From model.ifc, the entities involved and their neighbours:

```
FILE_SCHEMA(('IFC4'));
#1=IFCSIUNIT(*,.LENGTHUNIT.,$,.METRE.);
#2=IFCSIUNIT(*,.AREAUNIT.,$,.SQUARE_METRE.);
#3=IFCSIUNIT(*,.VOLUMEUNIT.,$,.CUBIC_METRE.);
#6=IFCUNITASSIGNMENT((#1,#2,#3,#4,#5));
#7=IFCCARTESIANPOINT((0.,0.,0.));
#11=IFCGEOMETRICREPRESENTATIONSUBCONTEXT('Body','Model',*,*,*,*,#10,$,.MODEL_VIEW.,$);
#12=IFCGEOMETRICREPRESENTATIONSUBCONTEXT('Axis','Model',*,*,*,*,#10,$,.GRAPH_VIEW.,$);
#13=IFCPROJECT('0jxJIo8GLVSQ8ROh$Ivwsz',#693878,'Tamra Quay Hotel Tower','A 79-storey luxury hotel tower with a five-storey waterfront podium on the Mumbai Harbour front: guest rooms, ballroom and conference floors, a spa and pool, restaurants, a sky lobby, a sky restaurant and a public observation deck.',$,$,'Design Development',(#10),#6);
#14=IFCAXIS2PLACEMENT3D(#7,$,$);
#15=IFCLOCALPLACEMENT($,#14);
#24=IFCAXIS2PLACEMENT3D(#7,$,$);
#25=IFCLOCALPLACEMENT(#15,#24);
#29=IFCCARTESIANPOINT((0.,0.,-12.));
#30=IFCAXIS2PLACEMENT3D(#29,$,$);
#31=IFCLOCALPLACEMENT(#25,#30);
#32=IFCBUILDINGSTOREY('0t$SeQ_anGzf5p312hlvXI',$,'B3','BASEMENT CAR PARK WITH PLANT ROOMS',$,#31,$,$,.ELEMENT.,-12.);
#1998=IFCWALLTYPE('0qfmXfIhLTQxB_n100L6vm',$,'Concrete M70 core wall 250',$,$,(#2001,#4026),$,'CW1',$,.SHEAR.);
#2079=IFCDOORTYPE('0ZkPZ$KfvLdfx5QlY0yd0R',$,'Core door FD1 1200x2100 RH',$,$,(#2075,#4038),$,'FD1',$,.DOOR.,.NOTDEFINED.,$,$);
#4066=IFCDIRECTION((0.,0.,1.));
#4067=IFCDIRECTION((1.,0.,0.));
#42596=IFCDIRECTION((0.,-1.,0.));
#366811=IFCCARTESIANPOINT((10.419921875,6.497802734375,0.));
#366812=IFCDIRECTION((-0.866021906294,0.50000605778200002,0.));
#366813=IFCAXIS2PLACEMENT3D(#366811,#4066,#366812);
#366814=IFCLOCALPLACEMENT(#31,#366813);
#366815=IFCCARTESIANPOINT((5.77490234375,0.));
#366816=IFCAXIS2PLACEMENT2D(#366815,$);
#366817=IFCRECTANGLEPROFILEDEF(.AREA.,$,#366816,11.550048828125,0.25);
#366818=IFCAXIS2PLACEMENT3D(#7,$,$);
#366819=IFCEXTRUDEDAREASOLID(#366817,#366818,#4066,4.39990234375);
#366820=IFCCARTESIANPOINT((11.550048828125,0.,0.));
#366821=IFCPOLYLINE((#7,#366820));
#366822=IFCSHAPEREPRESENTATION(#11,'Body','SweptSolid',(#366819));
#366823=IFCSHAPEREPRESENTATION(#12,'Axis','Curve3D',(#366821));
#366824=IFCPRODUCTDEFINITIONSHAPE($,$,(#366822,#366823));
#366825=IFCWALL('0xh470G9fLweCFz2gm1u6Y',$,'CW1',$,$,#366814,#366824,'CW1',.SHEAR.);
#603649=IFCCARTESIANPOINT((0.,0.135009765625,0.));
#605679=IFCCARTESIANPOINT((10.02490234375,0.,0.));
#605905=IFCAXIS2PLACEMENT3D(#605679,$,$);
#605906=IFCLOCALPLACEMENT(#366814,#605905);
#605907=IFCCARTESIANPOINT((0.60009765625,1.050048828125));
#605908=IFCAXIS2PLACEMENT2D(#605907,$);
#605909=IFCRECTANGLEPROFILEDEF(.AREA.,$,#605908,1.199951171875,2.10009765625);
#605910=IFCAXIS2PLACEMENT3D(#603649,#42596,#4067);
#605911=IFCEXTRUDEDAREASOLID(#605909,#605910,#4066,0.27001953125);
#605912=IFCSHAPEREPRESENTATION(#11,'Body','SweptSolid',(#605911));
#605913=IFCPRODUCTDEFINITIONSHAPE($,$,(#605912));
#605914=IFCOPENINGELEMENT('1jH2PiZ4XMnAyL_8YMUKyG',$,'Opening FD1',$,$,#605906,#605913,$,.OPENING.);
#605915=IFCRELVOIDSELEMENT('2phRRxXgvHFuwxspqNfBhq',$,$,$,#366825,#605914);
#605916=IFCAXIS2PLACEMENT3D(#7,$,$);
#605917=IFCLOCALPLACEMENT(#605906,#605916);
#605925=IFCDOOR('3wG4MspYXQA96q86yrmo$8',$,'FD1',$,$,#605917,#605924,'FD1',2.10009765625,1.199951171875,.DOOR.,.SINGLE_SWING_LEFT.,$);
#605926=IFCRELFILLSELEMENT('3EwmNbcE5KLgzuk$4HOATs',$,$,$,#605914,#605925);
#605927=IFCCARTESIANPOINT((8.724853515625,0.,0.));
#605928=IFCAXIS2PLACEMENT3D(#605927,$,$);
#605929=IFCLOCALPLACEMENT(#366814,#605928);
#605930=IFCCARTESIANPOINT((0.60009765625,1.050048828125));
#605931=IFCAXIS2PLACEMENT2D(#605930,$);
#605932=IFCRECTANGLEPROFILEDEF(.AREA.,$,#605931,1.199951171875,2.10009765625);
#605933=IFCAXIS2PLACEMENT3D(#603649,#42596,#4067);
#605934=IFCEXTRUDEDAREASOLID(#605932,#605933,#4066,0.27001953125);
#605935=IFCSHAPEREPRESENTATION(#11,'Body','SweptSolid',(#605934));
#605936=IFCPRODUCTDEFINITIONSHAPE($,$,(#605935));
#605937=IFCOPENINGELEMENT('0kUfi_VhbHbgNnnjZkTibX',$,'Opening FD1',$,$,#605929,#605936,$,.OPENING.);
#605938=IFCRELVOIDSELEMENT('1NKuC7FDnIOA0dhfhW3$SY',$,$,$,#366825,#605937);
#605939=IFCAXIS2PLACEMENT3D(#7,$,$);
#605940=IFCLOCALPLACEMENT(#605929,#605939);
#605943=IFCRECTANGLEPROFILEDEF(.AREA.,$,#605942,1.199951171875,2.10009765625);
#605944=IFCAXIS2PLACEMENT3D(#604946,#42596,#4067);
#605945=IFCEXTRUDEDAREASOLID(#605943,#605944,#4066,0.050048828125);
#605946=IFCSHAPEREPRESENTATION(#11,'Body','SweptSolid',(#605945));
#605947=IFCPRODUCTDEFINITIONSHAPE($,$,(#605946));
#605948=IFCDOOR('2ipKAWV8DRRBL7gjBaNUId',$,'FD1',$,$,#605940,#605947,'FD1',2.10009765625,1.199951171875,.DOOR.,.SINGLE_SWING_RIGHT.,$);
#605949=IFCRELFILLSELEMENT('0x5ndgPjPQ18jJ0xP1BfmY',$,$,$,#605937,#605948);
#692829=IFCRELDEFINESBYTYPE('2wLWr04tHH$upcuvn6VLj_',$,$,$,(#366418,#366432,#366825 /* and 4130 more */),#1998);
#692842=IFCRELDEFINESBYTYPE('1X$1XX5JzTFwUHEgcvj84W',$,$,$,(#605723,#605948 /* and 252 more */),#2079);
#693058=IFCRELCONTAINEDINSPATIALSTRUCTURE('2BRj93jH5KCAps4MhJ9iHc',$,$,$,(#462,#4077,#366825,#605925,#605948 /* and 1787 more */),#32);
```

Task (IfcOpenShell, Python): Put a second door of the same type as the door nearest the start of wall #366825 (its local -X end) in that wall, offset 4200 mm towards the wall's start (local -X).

```python
import ifcopenshell
import ifcopenshell.api.feature
import ifcopenshell.api.geometry
import ifcopenshell.api.root
import ifcopenshell.geom
import ifcopenshell.util.element
import ifcopenshell.util.placement
import ifcopenshell.util.shape
import ifcopenshell.util.unit

model = ifcopenshell.open("model.ifc")
unit_scale = ifcopenshell.util.unit.calculate_unit_scale(model)
settings = ifcopenshell.geom.settings()


def volume(element):
    """Net volume in cubic metres, openings subtracted."""
    shape = ifcopenshell.geom.create_shape(settings, element)
    return ifcopenshell.util.shape.get_volume(shape.geometry)


door = model.by_guid("2ipKAWV8DRRBL7gjBaNUId")
opening = door.FillsVoids[0].RelatingOpeningElement
wall = opening.VoidsElements[0].RelatingBuildingElement
before = volume(wall)
shift = ifcopenshell.util.placement.get_local_placement(wall.ObjectPlacement)[:3, 0] * -4.2 / unit_scale

# copy_class copies the void relationship, type, container and properties, but no geometry.
new_opening = ifcopenshell.api.root.copy_class(model, product=opening)
new_opening.Representation = ifcopenshell.util.element.copy_deep(
    model, opening.Representation, exclude=["IfcGeometricRepresentationContext", "IfcRepresentationMap"]
)
new_door = ifcopenshell.api.root.copy_class(model, product=door)
new_door.Representation = ifcopenshell.util.element.copy_deep(
    model, door.Representation, exclude=["IfcGeometricRepresentationContext", "IfcRepresentationMap"]
)
new_door.Tag = None
ifcopenshell.api.feature.add_filling(model, opening=new_opening, element=new_door)

for old, new in ((opening, new_opening), (door, new_door)):
    matrix = ifcopenshell.util.placement.get_local_placement(old.ObjectPlacement)
    matrix[:3, 3] += shift
    ifcopenshell.api.geometry.edit_object_placement(model, product=new, matrix=matrix, is_si=False)

after = volume(wall)

print(f"wall volume {before:.3f} -> {after:.3f} m3")

model.write("model_updated.ifc")
```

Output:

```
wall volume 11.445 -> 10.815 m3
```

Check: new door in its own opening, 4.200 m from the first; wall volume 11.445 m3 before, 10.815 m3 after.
